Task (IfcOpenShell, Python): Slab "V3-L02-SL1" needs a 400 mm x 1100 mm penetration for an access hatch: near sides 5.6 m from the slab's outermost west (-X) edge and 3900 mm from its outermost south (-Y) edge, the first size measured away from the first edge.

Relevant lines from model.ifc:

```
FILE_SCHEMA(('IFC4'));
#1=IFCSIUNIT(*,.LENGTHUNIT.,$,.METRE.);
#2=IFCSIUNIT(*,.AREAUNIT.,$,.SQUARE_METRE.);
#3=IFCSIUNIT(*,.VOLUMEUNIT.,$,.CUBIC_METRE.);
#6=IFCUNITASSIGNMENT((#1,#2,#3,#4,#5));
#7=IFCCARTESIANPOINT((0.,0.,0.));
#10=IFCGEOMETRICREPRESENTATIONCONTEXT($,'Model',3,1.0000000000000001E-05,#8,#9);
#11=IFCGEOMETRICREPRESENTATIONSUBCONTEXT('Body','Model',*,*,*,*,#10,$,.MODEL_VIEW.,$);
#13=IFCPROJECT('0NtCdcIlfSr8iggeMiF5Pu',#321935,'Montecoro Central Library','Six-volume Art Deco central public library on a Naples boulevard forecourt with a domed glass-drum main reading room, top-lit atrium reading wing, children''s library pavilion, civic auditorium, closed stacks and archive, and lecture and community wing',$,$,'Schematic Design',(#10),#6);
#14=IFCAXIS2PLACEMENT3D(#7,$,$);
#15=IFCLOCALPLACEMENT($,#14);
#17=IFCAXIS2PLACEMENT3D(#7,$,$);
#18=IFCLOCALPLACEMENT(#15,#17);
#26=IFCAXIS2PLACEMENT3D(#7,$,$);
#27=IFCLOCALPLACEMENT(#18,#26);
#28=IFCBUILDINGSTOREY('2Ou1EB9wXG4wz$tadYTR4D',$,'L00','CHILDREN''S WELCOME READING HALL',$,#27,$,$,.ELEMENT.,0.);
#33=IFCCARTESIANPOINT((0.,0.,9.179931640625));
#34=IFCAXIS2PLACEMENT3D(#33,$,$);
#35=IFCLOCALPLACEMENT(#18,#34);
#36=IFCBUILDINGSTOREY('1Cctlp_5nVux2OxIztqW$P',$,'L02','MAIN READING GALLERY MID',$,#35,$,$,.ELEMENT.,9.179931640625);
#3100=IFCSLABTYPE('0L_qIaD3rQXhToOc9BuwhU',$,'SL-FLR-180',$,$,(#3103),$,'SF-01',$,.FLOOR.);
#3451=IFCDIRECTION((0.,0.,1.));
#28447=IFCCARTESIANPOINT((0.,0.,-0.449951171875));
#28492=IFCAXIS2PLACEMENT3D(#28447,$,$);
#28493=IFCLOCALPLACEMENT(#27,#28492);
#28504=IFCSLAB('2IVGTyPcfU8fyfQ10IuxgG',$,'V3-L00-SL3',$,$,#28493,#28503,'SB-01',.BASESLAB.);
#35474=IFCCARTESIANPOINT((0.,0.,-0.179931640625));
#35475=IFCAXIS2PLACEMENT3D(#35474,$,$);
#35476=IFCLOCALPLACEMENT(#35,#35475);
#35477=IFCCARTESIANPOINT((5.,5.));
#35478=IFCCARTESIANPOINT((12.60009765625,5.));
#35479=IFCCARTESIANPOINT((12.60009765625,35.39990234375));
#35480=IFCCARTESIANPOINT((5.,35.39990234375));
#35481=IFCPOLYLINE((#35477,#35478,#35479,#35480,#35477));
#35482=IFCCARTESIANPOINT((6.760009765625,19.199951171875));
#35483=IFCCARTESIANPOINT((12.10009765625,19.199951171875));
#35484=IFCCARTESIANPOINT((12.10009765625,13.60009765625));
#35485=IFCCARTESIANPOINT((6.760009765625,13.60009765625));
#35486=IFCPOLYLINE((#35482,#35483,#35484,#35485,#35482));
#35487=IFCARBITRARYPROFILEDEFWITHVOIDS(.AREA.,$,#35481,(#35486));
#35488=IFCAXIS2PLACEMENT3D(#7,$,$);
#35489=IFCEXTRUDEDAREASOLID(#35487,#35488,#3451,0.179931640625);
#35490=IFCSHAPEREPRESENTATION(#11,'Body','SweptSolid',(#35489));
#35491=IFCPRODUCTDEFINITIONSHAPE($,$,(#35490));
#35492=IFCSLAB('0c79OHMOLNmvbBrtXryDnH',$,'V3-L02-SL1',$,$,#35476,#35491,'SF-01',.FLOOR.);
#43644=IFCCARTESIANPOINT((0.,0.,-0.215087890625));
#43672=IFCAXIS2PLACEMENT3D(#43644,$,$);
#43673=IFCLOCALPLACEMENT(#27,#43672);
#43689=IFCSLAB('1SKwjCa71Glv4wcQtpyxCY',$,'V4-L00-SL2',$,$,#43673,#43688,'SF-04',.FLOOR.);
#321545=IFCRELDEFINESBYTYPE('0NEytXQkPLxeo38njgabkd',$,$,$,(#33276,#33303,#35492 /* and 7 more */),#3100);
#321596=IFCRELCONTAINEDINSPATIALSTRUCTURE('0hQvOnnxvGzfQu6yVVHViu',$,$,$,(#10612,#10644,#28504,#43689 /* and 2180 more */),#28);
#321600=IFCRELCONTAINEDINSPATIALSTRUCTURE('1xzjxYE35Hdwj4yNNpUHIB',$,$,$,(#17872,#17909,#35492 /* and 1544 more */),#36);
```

```python
import numpy as np
import ifcopenshell
import ifcopenshell.api.feature
import ifcopenshell.api.geometry
import ifcopenshell.api.root
import ifcopenshell.geom
import ifcopenshell.util.placement
import ifcopenshell.util.representation
import ifcopenshell.util.shape
import ifcopenshell.util.unit

model = ifcopenshell.open("model.ifc")
unit_scale = ifcopenshell.util.unit.calculate_unit_scale(model)
settings = ifcopenshell.geom.settings()


def volume(element):
    """Net volume in cubic metres, openings subtracted."""
    shape = ifcopenshell.geom.create_shape(settings, element)
    return ifcopenshell.util.shape.get_volume(shape.geometry)


slab = model.by_guid("0c79OHMOLNmvbBrtXryDnH")
before = volume(slab)

# Extent in the slab's own axes, in metres. The edges named are its -X and -Y sides.
slab_shape = ifcopenshell.geom.create_shape(settings, slab)
vertices = ifcopenshell.util.shape.get_vertices(slab_shape.geometry)
x_min, y_min, bottom = vertices.min(axis=0)
top = vertices[:, 2].max()

opening = ifcopenshell.api.root.create_entity(model, ifc_class="IfcOpeningElement", name="Access hatch opening", predefined_type="OPENING")
context = ifcopenshell.util.representation.get_context(model, "Model", "Body", "MODEL_VIEW")
width, depth = 0.4, 1.1
outline = [(0.0, 0.0), (width, 0.0), (width, depth), (0.0, depth), (0.0, 0.0)]
# Overshoot both faces by 50 mm so the cut is clean.
shape = ifcopenshell.api.geometry.add_slab_representation(
    model, context=context, depth=top - bottom + 0.1, polyline=outline
)
ifcopenshell.api.geometry.assign_representation(model, product=opening, representation=shape)

matrix = ifcopenshell.util.placement.get_local_placement(slab.ObjectPlacement)
matrix[:, 3] = matrix @ np.append(np.array([x_min + 5.6, y_min + 3.9, bottom - 0.05]) / unit_scale, 1.0)
ifcopenshell.api.geometry.edit_object_placement(model, product=opening, matrix=matrix, is_si=False)
ifcopenshell.api.feature.add_feature(model, feature=opening, element=slab)

after = volume(slab)

print(f"slab volume {before:.3f} -> {after:.3f} m3")

model.write("model-out.ifc")
```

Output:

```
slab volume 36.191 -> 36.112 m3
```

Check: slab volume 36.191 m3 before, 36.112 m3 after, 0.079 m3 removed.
